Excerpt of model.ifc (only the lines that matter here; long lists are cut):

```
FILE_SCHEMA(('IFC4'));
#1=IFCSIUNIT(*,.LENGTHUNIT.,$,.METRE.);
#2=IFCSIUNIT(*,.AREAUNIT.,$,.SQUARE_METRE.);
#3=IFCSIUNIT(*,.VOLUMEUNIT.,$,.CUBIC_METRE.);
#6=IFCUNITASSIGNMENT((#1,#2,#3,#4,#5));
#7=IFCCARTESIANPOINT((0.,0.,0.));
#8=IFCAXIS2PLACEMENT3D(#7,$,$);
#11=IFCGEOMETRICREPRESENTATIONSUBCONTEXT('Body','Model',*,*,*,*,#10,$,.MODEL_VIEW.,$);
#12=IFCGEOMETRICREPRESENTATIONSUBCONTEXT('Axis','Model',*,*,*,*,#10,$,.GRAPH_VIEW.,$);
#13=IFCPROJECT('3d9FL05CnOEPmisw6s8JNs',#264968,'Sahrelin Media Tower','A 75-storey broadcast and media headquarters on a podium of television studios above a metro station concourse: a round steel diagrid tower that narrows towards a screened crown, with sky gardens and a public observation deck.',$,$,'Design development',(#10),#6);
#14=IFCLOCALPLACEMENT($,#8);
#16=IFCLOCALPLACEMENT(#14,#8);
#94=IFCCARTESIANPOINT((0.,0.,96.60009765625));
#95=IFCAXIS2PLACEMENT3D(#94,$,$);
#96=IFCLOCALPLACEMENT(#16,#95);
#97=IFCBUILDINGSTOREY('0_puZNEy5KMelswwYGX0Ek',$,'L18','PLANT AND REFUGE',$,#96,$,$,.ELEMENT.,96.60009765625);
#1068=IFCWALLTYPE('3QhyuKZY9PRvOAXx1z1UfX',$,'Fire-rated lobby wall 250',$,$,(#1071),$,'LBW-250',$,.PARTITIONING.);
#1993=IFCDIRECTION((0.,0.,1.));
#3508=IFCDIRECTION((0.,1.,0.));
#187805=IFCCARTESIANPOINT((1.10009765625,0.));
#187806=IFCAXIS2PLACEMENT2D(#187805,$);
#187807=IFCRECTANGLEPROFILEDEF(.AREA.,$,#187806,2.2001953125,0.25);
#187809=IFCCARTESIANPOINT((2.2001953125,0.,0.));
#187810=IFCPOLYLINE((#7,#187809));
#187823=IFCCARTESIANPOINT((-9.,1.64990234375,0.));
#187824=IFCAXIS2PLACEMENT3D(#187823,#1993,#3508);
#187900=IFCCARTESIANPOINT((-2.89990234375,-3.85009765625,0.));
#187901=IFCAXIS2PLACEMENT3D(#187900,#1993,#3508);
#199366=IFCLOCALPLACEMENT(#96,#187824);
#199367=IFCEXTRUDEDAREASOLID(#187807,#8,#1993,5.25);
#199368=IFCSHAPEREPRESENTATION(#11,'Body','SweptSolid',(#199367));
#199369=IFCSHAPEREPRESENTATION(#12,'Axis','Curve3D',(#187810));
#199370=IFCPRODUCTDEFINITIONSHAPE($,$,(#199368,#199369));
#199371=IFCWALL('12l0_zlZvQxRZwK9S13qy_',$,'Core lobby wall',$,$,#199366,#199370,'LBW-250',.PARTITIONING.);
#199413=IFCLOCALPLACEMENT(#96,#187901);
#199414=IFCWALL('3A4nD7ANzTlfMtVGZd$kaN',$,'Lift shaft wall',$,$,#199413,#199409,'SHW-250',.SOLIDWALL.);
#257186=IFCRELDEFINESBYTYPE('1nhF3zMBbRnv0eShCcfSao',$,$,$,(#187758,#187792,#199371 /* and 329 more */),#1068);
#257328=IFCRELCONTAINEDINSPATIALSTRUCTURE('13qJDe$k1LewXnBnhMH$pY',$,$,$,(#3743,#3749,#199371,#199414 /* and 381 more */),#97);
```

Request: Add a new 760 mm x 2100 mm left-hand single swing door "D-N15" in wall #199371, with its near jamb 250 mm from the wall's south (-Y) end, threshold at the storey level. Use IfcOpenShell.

```python
import numpy as np
import ifcopenshell
import ifcopenshell.api.feature
import ifcopenshell.api.geometry
import ifcopenshell.api.root
import ifcopenshell.api.spatial
import ifcopenshell.geom
import ifcopenshell.util.element
import ifcopenshell.util.placement
import ifcopenshell.util.representation
import ifcopenshell.util.shape
import ifcopenshell.util.unit

model = ifcopenshell.open("model.ifc")
unit_scale = ifcopenshell.util.unit.calculate_unit_scale(model)
settings = ifcopenshell.geom.settings()


def volume(element):
    """Net volume in cubic metres, openings subtracted."""
    shape = ifcopenshell.geom.create_shape(settings, element)
    return ifcopenshell.util.shape.get_volume(shape.geometry)


wall = model.by_id(199371)
storey = ifcopenshell.util.element.get_container(wall, ifc_class="IfcBuildingStorey")
context = ifcopenshell.util.representation.get_context(model, "Model", "Body", "MODEL_VIEW")
before = volume(wall)

width, height, from_end, sill = 0.76, 2.1, 0.25, 0.0  # metres

# The wall runs along its own X axis, and the end named is its -X end.
wall_shape = ifcopenshell.geom.create_shape(settings, wall)
x, y, z = ifcopenshell.util.shape.get_vertices(wall_shape.geometry).T
start = x.min() + from_end
face, thickness = float(y.min()), float(y.max() - y.min())
wall_matrix = ifcopenshell.util.placement.get_local_placement(wall.ObjectPlacement)
level = ifcopenshell.util.placement.get_local_placement(storey.ObjectPlacement)[2, 3]


def in_wall(x, y):
    """Placement at x, y metres in the wall's axes, at sill height."""
    matrix = wall_matrix.copy()
    matrix[:, 3] = wall_matrix @ np.array([x / unit_scale, y / unit_scale, 0.0, 1.0])
    matrix[2, 3] = level + sill / unit_scale
    return matrix


# Opening: a box that overshoots both wall faces by 50 mm.
opening = ifcopenshell.api.root.create_entity(model, ifc_class="IfcOpeningElement", predefined_type="OPENING")
box = ifcopenshell.api.geometry.add_wall_representation(
    model, context=context, length=width, height=height, thickness=thickness + 0.1
)
ifcopenshell.api.geometry.assign_representation(model, product=opening, representation=box)
ifcopenshell.api.geometry.edit_object_placement(model, product=opening, matrix=in_wall(start, face - 0.05), is_si=False)
ifcopenshell.api.feature.add_feature(model, feature=opening, element=wall)

door = ifcopenshell.api.root.create_entity(model, ifc_class="IfcDoor", name="D-N15", predefined_type="DOOR")
door.OverallWidth, door.OverallHeight = width / unit_scale, height / unit_scale
door.OperationType = "SINGLE_SWING_LEFT"
body = ifcopenshell.api.geometry.add_door_representation(
    model,
    context=context,
    overall_width=door.OverallWidth,
    overall_height=door.OverallHeight,
    operation_type="SINGLE_SWING_LEFT",
    lining_properties={"LiningDepth": thickness / unit_scale, "ThresholdDepth": thickness / unit_scale},
)
ifcopenshell.api.geometry.assign_representation(model, product=door, representation=body)
ifcopenshell.api.spatial.assign_container(model, products=[door], relating_structure=storey)
ifcopenshell.api.feature.add_filling(model, opening=opening, element=door)

# The lining spans the wall, so the door starts at the wall face.
ifcopenshell.api.geometry.edit_object_placement(model, product=door, matrix=in_wall(start, face), is_si=False)

after = volume(wall)

print(f"wall volume {before:.3f} -> {after:.3f} m3")

model.write("model_rev.ifc")
```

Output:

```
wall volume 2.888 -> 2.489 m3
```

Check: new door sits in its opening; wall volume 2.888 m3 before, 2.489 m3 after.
